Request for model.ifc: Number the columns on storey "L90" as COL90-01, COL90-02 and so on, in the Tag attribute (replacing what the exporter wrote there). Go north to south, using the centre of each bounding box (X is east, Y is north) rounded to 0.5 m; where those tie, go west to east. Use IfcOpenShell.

First a look at what the model holds.

```python
import ifcopenshell
import ifcopenshell.util.element
import ifcopenshell.util.placement

model = ifcopenshell.open("model.ifc")
print(model.schema)
storey = next(s for s in model.by_type("IfcBuildingStorey") if s.Name == "L90")
columns = [e for e in ifcopenshell.util.element.get_decomposition(storey) if e.is_a("IfcColumn")]
for e in sorted(columns, key=lambda e: e.id()):
    origin = ifcopenshell.util.placement.get_local_placement(e.ObjectPlacement)[:3, 3]
    print(e.id(), e.Tag, e.Name, origin.round(2) + 0.0, sep=" | ")
```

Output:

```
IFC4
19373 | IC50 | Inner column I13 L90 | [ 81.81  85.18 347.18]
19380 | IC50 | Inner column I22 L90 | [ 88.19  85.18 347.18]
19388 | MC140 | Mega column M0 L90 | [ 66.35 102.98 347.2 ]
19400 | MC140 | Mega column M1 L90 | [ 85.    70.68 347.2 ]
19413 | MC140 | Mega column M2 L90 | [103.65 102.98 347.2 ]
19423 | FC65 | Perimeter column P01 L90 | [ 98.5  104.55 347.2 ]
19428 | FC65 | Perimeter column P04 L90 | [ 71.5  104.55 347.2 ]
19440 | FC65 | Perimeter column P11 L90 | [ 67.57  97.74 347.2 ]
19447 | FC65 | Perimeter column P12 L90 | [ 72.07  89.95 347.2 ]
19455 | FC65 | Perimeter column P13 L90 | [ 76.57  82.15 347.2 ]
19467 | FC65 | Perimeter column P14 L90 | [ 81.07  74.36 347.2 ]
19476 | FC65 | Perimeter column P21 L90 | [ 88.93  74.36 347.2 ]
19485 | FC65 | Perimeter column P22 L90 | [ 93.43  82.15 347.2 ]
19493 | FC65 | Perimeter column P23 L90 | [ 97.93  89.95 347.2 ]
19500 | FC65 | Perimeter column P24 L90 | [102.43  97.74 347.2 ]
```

```python
import ifcopenshell
import ifcopenshell.geom
import ifcopenshell.util.element
import ifcopenshell.util.shape

model = ifcopenshell.open("model.ifc")
settings = ifcopenshell.geom.settings()
settings.set("use-world-coords", True)


def centre(element):
    shape = ifcopenshell.geom.create_shape(settings, element)
    return ifcopenshell.util.shape.get_bbox_centroid(shape.geometry)


storey = next(s for s in model.by_type("IfcBuildingStorey") if s.Name == "L90")
columns = [e for e in ifcopenshell.util.element.get_decomposition(storey) if e.is_a("IfcColumn")]

# Insertion points can sit at a corner or the storey origin, so sort by the geometry (in metres).
centres = {e: centre(e) for e in columns}
columns.sort(key=lambda e: (-round(centres[e][1] / 0.5), centres[e][0]))

for i, e in enumerate(columns, start=1):
    number = f"COL90-{i:02d}"
    e.Tag = number
    print(e.id(), number)

model.write("model_edited.ifc")
```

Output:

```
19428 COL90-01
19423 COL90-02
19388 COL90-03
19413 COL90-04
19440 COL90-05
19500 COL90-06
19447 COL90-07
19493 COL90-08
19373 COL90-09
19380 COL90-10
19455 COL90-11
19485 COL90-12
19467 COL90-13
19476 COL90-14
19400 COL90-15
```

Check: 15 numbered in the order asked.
